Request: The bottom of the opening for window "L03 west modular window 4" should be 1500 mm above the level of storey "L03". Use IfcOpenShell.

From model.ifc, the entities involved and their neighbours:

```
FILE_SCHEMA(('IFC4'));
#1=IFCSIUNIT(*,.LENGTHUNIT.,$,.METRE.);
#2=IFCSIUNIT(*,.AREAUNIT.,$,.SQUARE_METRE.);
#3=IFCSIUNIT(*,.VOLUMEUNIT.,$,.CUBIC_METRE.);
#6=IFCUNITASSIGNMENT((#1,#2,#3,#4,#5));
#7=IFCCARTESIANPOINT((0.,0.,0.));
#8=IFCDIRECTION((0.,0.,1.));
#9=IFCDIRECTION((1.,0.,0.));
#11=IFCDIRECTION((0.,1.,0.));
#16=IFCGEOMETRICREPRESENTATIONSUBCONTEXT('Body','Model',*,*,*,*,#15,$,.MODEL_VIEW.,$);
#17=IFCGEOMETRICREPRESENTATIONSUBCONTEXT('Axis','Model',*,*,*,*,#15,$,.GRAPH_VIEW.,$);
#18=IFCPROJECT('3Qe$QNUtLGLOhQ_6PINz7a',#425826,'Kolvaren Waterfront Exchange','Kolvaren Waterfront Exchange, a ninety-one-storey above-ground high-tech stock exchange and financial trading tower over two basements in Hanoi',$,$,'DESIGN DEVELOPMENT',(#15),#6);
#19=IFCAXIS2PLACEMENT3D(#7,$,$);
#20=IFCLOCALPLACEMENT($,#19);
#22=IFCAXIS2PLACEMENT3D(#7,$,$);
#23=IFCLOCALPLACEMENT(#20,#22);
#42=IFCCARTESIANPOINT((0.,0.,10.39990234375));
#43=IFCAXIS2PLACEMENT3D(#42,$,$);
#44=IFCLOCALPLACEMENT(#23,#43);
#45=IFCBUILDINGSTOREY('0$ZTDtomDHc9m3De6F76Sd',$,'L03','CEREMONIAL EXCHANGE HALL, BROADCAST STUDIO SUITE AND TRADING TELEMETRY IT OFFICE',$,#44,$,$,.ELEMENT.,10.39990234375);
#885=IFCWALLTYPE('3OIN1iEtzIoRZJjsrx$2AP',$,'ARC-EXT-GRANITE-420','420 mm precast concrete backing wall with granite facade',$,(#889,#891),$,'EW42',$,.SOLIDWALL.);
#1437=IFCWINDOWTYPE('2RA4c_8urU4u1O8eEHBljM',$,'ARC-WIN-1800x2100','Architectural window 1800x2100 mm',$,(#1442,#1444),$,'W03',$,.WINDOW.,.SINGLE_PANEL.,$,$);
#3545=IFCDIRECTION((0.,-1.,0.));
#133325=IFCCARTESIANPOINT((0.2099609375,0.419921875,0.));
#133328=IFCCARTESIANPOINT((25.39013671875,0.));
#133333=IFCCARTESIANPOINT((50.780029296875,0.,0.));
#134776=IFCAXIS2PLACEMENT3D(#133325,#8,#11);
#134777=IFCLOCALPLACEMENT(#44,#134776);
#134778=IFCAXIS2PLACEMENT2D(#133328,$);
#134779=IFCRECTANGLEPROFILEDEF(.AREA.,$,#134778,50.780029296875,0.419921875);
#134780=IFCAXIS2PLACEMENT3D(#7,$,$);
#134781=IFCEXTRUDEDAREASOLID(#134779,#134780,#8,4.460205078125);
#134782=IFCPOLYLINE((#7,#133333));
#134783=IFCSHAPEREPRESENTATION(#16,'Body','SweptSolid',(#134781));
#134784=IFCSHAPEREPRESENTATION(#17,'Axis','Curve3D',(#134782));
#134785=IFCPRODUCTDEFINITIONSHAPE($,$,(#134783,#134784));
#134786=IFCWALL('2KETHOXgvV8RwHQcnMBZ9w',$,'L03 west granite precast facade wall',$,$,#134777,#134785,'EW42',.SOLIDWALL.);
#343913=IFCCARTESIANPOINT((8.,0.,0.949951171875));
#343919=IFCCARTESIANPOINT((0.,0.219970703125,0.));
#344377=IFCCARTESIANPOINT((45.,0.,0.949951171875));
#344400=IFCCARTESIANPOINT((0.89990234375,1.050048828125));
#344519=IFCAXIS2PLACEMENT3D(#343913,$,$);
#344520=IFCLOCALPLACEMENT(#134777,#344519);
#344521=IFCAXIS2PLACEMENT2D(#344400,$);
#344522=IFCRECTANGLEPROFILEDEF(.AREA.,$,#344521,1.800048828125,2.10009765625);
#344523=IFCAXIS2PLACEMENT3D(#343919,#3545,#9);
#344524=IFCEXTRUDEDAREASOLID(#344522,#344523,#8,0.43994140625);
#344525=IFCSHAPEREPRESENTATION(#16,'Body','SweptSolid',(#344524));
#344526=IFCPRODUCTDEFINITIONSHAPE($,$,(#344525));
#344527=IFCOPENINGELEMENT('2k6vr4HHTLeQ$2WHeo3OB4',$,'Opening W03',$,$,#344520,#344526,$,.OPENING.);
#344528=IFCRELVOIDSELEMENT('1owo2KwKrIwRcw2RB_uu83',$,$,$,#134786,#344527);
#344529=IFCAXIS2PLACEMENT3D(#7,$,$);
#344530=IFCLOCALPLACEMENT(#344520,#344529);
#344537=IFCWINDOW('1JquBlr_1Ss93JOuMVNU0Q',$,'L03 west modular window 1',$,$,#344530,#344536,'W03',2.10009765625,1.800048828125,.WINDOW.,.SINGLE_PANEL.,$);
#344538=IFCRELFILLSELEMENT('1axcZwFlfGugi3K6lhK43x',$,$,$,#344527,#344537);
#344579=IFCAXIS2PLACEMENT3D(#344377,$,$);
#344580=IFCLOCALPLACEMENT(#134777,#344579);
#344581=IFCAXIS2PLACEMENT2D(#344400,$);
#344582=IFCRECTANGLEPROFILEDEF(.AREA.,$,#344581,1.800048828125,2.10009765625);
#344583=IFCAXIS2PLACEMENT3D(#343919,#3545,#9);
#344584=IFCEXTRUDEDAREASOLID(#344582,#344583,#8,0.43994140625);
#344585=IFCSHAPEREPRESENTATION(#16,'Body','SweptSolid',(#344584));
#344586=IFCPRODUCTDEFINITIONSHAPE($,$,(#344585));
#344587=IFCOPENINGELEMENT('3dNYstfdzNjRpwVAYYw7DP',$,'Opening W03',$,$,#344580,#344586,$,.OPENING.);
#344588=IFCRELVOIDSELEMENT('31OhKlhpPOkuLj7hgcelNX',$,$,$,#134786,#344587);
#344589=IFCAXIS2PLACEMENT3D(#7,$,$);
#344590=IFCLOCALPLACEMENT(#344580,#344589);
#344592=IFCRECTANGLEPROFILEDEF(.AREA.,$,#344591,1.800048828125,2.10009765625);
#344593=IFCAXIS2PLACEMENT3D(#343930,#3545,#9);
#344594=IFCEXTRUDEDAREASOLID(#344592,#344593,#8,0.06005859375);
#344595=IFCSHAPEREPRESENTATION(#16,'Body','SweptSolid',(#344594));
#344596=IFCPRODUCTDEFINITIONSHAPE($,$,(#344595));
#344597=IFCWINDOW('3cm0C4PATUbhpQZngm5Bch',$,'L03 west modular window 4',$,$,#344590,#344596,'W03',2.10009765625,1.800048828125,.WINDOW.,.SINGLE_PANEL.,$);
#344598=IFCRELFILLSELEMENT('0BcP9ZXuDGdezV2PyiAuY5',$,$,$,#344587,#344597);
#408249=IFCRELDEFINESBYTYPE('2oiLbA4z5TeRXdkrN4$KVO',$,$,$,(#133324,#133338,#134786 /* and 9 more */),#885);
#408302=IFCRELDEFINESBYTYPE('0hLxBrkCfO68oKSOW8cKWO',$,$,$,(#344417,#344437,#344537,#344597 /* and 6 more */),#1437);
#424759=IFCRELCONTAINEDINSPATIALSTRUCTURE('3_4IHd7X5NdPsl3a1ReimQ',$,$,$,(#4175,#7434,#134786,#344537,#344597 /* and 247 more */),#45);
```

```python
import numpy as np
import ifcopenshell
import ifcopenshell.api.geometry
import ifcopenshell.geom
import ifcopenshell.util.element
import ifcopenshell.util.placement
import ifcopenshell.util.shape
import ifcopenshell.util.unit

model = ifcopenshell.open("model.ifc")
unit_scale = ifcopenshell.util.unit.calculate_unit_scale(model)

window = model.by_id(344597)
opening = window.FillsVoids[0].RelatingOpeningElement
storey = ifcopenshell.util.element.get_container(window, ifc_class="IfcBuildingStorey")
level = ifcopenshell.util.placement.get_local_placement(storey.ObjectPlacement)[2, 3]

# The opening's origin need not be at the sill, so measure its lowest point.
shape = ifcopenshell.geom.create_shape(ifcopenshell.geom.settings(), opening)
bottom = ifcopenshell.util.shape.get_shape_bottom_elevation(shape, shape.geometry) / unit_scale
dz = level + 1.5 / unit_scale - bottom

shift = np.array([0.0, 0.0, dz])
# The window is placed relative to its opening, so it follows when the opening moves.
matrix = ifcopenshell.util.placement.get_local_placement(opening.ObjectPlacement)
matrix[:3, 3] += shift
ifcopenshell.api.geometry.edit_object_placement(
    model, product=opening, matrix=matrix, is_si=False, should_transform_children=True
)

print(f"moved by {dz * unit_scale:+.3f} m")

model.write("model_rev.ifc")
```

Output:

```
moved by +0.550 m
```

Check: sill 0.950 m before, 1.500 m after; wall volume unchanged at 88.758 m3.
